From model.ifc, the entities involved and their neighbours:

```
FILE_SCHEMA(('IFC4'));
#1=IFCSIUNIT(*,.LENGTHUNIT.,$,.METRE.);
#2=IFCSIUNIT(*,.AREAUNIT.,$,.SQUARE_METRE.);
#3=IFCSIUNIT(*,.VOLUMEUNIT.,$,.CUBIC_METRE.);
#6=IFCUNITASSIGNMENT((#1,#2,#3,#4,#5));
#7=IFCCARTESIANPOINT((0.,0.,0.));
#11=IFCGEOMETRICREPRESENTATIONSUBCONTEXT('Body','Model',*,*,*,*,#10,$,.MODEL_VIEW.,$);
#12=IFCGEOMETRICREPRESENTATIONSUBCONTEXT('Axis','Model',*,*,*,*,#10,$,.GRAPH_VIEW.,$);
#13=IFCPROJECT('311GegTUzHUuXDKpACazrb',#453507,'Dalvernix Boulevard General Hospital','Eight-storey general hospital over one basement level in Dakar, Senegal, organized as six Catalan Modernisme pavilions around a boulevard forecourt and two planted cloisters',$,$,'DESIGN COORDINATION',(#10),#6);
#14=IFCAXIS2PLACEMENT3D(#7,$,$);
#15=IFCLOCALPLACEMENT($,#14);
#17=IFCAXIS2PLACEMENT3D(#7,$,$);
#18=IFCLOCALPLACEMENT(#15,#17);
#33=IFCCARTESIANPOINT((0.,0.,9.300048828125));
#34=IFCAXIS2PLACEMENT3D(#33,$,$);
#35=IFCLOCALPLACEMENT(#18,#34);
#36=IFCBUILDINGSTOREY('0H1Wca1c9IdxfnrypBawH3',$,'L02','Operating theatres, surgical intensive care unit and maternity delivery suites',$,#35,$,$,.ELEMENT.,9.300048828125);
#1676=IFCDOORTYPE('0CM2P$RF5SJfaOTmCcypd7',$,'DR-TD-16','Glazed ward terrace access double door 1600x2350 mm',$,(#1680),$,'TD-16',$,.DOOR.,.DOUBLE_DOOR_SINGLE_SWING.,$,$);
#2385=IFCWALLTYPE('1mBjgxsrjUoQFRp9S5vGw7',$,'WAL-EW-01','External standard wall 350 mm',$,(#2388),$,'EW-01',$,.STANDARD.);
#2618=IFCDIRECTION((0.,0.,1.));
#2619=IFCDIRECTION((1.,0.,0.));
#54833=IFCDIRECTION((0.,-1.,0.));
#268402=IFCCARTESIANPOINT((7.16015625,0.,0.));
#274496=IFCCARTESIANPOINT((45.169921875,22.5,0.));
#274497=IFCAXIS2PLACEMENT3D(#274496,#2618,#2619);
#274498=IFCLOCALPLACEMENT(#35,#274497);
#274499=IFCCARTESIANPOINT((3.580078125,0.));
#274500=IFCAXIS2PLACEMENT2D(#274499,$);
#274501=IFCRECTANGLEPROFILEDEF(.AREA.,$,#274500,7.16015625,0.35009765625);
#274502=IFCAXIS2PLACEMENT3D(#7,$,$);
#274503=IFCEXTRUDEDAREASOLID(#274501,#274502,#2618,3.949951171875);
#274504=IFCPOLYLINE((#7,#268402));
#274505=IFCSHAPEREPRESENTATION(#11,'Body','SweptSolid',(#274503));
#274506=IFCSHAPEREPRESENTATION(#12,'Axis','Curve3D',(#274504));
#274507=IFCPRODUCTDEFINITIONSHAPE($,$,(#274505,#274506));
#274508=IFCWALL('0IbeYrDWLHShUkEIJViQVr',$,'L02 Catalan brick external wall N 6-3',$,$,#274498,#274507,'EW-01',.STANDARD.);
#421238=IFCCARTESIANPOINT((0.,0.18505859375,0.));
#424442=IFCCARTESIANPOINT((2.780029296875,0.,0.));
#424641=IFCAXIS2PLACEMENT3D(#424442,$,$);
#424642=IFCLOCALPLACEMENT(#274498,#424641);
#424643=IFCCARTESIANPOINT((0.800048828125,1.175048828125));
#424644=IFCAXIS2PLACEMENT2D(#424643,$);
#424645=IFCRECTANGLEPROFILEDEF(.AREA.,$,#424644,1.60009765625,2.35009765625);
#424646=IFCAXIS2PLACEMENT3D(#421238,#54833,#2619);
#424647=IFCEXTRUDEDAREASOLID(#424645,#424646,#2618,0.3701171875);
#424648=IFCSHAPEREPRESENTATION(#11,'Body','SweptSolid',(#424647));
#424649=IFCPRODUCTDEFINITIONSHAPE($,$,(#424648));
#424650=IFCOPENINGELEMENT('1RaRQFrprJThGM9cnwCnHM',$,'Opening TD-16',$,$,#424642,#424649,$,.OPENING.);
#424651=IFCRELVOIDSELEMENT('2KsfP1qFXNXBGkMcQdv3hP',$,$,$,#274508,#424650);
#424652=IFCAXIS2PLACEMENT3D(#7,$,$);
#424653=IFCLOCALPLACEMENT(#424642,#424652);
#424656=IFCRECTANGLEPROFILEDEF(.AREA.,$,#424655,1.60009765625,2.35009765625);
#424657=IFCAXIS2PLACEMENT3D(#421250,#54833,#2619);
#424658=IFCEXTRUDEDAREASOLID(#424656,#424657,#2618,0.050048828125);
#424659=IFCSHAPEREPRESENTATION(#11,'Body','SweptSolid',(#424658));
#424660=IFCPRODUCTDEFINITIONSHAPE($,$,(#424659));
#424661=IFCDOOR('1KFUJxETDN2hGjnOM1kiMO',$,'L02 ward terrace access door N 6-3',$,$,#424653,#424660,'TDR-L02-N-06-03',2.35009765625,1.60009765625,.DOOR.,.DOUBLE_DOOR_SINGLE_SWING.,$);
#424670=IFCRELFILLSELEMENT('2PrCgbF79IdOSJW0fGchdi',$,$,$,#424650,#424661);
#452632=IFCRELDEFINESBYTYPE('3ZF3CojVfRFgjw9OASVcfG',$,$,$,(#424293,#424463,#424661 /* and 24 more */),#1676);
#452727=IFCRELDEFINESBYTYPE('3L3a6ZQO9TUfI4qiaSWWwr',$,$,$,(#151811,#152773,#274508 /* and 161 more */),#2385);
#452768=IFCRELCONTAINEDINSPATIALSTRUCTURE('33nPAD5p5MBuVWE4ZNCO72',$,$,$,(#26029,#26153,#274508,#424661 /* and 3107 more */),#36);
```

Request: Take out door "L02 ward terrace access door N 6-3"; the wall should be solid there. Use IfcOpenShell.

```python
import ifcopenshell
import ifcopenshell.api.feature
import ifcopenshell.api.root
import ifcopenshell.geom
import ifcopenshell.util.shape

model = ifcopenshell.open("model.ifc")
settings = ifcopenshell.geom.settings()


def volume(element):
    """Net volume in cubic metres, openings subtracted."""
    shape = ifcopenshell.geom.create_shape(settings, element)
    return ifcopenshell.util.shape.get_volume(shape.geometry)


door = model.by_id(424661)
opening = door.FillsVoids[0].RelatingOpeningElement
wall = opening.VoidsElements[0].RelatingBuildingElement
before = volume(wall)

ifcopenshell.api.root.remove_product(model, product=door)
ifcopenshell.api.feature.remove_feature(model, feature=opening)

after = volume(wall)

print(f"wall volume {before:.3f} -> {after:.3f} m3")

model.write("model_updated.ifc")
```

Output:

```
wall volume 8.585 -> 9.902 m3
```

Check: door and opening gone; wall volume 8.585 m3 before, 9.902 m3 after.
